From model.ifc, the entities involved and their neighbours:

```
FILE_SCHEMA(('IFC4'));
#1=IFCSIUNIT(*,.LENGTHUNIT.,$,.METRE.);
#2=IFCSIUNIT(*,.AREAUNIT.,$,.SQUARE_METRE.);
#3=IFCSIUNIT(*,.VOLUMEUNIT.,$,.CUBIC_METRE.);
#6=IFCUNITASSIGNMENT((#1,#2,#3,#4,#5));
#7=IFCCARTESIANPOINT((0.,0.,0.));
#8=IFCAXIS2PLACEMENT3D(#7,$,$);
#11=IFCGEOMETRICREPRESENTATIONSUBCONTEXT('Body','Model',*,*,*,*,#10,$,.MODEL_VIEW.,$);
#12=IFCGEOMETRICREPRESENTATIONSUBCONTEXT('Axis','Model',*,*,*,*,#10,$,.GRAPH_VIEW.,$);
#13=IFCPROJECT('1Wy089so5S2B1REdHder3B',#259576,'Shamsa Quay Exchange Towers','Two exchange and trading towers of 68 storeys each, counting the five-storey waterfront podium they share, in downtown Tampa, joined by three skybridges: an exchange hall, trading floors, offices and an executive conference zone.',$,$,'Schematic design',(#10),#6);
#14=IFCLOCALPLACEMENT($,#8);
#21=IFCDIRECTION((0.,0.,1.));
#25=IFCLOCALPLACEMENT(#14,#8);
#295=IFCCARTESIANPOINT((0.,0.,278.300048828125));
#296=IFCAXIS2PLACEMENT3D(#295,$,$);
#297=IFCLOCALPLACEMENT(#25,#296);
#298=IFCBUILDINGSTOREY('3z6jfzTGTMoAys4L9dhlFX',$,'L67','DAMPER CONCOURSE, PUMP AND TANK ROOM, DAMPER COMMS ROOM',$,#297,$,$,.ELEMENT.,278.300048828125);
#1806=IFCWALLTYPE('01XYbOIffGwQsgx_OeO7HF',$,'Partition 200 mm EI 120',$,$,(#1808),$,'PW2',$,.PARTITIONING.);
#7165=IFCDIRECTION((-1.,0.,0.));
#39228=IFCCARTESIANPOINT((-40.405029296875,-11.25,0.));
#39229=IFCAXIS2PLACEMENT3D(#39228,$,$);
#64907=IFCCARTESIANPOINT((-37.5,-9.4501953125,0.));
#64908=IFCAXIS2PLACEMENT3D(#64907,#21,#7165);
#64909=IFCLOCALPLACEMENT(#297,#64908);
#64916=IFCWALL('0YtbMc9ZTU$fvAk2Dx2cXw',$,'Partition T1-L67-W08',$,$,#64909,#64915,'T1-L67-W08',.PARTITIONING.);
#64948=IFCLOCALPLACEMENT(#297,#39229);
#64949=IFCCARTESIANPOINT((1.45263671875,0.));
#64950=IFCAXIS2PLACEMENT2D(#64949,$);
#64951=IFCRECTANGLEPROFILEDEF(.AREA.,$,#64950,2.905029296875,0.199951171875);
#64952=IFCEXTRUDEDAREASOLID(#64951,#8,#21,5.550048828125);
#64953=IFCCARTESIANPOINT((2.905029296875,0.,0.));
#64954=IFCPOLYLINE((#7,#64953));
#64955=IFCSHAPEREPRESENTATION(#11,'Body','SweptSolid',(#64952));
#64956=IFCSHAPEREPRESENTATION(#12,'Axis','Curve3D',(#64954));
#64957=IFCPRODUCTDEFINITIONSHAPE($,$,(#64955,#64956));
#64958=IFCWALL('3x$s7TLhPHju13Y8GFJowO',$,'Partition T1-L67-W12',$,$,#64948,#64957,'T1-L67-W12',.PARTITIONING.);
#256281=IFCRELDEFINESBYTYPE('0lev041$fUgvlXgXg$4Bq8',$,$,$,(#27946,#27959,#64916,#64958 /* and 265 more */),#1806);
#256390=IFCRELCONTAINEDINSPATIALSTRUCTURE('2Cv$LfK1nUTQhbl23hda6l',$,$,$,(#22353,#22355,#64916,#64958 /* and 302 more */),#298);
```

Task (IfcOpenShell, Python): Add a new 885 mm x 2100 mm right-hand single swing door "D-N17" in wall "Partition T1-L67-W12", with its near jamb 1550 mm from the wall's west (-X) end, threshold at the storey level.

```python
import numpy as np
import ifcopenshell
import ifcopenshell.api.feature
import ifcopenshell.api.geometry
import ifcopenshell.api.root
import ifcopenshell.api.spatial
import ifcopenshell.geom
import ifcopenshell.util.element
import ifcopenshell.util.placement
import ifcopenshell.util.representation
import ifcopenshell.util.shape
import ifcopenshell.util.unit

model = ifcopenshell.open("model.ifc")
unit_scale = ifcopenshell.util.unit.calculate_unit_scale(model)
settings = ifcopenshell.geom.settings()


def volume(element):
    """Net volume in cubic metres, openings subtracted."""
    shape = ifcopenshell.geom.create_shape(settings, element)
    return ifcopenshell.util.shape.get_volume(shape.geometry)


wall = model.by_id(64958)
storey = ifcopenshell.util.element.get_container(wall, ifc_class="IfcBuildingStorey")
context = ifcopenshell.util.representation.get_context(model, "Model", "Body", "MODEL_VIEW")
before = volume(wall)

width, height, from_end, sill = 0.885, 2.1, 1.55, 0.0  # metres

# The wall runs along its own X axis, and the end named is its -X end.
wall_shape = ifcopenshell.geom.create_shape(settings, wall)
x, y, z = ifcopenshell.util.shape.get_vertices(wall_shape.geometry).T
start = x.min() + from_end
face, thickness = float(y.min()), float(y.max() - y.min())
wall_matrix = ifcopenshell.util.placement.get_local_placement(wall.ObjectPlacement)
level = ifcopenshell.util.placement.get_local_placement(storey.ObjectPlacement)[2, 3]


def in_wall(x, y):
    """Placement at x, y metres in the wall's axes, at sill height."""
    matrix = wall_matrix.copy()
    matrix[:, 3] = wall_matrix @ np.array([x / unit_scale, y / unit_scale, 0.0, 1.0])
    matrix[2, 3] = level + sill / unit_scale
    return matrix


# Opening: a box that overshoots both wall faces by 50 mm.
opening = ifcopenshell.api.root.create_entity(model, ifc_class="IfcOpeningElement", predefined_type="OPENING")
box = ifcopenshell.api.geometry.add_wall_representation(
    model, context=context, length=width, height=height, thickness=thickness + 0.1
)
ifcopenshell.api.geometry.assign_representation(model, product=opening, representation=box)
ifcopenshell.api.geometry.edit_object_placement(model, product=opening, matrix=in_wall(start, face - 0.05), is_si=False)
ifcopenshell.api.feature.add_feature(model, feature=opening, element=wall)

door = ifcopenshell.api.root.create_entity(model, ifc_class="IfcDoor", name="D-N17", predefined_type="DOOR")
door.OverallWidth, door.OverallHeight = width / unit_scale, height / unit_scale
door.OperationType = "SINGLE_SWING_RIGHT"
body = ifcopenshell.api.geometry.add_door_representation(
    model,
    context=context,
    overall_width=door.OverallWidth,
    overall_height=door.OverallHeight,
    operation_type="SINGLE_SWING_RIGHT",
    lining_properties={"LiningDepth": thickness / unit_scale, "ThresholdDepth": thickness / unit_scale},
)
ifcopenshell.api.geometry.assign_representation(model, product=door, representation=body)
ifcopenshell.api.spatial.assign_container(model, products=[door], relating_structure=storey)
ifcopenshell.api.feature.add_filling(model, opening=opening, element=door)

# The lining spans the wall, so the door starts at the wall face.
ifcopenshell.api.geometry.edit_object_placement(model, product=door, matrix=in_wall(start, face), is_si=False)

after = volume(wall)

print(f"wall volume {before:.3f} -> {after:.3f} m3")

model.write("model-out.ifc")
```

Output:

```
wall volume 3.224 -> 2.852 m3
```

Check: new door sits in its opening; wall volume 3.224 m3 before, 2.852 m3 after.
